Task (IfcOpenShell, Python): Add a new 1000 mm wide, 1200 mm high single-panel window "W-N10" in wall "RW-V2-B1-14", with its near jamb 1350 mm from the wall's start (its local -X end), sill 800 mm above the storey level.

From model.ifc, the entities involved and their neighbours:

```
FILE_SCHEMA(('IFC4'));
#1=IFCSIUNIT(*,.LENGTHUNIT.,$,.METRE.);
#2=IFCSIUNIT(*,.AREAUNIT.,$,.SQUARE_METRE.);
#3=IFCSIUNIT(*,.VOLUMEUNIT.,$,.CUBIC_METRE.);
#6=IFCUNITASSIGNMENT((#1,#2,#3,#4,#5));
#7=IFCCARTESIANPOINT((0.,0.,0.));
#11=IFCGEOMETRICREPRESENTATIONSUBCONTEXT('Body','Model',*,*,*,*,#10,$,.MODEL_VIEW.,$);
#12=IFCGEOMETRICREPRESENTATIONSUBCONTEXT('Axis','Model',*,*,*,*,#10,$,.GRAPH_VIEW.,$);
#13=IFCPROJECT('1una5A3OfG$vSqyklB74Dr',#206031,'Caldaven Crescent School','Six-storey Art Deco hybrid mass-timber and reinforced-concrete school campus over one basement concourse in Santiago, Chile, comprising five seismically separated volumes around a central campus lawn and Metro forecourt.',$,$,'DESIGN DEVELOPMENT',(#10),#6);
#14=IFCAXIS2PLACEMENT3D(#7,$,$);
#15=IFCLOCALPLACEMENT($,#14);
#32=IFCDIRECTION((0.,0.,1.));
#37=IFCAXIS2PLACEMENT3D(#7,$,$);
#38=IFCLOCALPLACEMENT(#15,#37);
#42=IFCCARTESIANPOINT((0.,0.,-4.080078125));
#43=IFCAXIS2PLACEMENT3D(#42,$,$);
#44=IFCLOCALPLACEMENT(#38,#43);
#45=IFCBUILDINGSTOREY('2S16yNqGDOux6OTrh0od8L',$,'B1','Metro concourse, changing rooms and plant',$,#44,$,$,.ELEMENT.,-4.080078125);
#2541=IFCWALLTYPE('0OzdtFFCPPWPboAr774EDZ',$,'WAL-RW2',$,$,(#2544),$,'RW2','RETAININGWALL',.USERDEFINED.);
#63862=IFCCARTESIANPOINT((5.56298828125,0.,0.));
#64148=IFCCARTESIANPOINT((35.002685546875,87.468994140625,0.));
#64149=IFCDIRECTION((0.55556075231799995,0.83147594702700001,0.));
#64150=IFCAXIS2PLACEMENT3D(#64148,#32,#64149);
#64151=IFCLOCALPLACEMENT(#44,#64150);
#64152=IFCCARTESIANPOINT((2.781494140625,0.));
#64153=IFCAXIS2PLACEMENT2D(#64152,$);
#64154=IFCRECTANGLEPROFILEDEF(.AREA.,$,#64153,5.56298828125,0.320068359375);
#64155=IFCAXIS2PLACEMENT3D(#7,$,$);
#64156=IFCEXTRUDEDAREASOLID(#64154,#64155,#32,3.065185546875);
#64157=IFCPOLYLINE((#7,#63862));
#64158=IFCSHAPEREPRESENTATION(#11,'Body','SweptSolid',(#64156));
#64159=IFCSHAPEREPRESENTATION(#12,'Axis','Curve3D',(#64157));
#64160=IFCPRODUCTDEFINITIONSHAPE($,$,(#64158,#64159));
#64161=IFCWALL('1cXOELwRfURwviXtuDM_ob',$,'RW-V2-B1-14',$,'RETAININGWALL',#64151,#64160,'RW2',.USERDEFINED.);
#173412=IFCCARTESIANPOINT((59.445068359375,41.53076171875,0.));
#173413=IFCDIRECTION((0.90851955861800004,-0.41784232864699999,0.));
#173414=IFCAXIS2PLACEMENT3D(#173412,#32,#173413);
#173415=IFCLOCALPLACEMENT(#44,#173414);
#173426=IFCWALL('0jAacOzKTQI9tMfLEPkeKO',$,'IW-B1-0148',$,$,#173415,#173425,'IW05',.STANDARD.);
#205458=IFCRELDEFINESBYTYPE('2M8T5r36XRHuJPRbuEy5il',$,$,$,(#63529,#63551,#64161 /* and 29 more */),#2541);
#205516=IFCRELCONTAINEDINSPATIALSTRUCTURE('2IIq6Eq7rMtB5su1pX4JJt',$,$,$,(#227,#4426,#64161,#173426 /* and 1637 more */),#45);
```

```python
import numpy as np
import ifcopenshell
import ifcopenshell.api.feature
import ifcopenshell.api.geometry
import ifcopenshell.api.root
import ifcopenshell.api.spatial
import ifcopenshell.geom
import ifcopenshell.util.element
import ifcopenshell.util.placement
import ifcopenshell.util.representation
import ifcopenshell.util.shape
import ifcopenshell.util.unit

model = ifcopenshell.open("model.ifc")
unit_scale = ifcopenshell.util.unit.calculate_unit_scale(model)
settings = ifcopenshell.geom.settings()


def volume(element):
    """Net volume in cubic metres, openings subtracted."""
    shape = ifcopenshell.geom.create_shape(settings, element)
    return ifcopenshell.util.shape.get_volume(shape.geometry)


wall = model.by_guid("1cXOELwRfURwviXtuDM_ob")
storey = ifcopenshell.util.element.get_container(wall, ifc_class="IfcBuildingStorey")
context = ifcopenshell.util.representation.get_context(model, "Model", "Body", "MODEL_VIEW")
before = volume(wall)

width, height, from_end, sill = 1, 1.2, 1.35, 0.8  # metres

# The wall runs along its own X axis, and the end named is its -X end.
wall_shape = ifcopenshell.geom.create_shape(settings, wall)
x, y, z = ifcopenshell.util.shape.get_vertices(wall_shape.geometry).T
start = x.min() + from_end
face, thickness = float(y.min()), float(y.max() - y.min())
wall_matrix = ifcopenshell.util.placement.get_local_placement(wall.ObjectPlacement)
level = ifcopenshell.util.placement.get_local_placement(storey.ObjectPlacement)[2, 3]


def in_wall(x, y):
    """Placement at x, y metres in the wall's axes, at sill height."""
    matrix = wall_matrix.copy()
    matrix[:, 3] = wall_matrix @ np.array([x / unit_scale, y / unit_scale, 0.0, 1.0])
    matrix[2, 3] = level + sill / unit_scale
    return matrix


# Opening: a box that overshoots both wall faces by 50 mm.
opening = ifcopenshell.api.root.create_entity(model, ifc_class="IfcOpeningElement", predefined_type="OPENING")
box = ifcopenshell.api.geometry.add_wall_representation(
    model, context=context, length=width, height=height, thickness=thickness + 0.1
)
ifcopenshell.api.geometry.assign_representation(model, product=opening, representation=box)
ifcopenshell.api.geometry.edit_object_placement(model, product=opening, matrix=in_wall(start, face - 0.05), is_si=False)
ifcopenshell.api.feature.add_feature(model, feature=opening, element=wall)

window = ifcopenshell.api.root.create_entity(model, ifc_class="IfcWindow", name="W-N10", predefined_type="WINDOW")
window.OverallWidth, window.OverallHeight = width / unit_scale, height / unit_scale
window.PartitioningType = "SINGLE_PANEL"
body = ifcopenshell.api.geometry.add_window_representation(
    model,
    context=context,
    overall_width=window.OverallWidth,
    overall_height=window.OverallHeight,
    partition_type="SINGLE_PANEL",
)
ifcopenshell.api.geometry.assign_representation(model, product=window, representation=body)
ifcopenshell.api.spatial.assign_container(model, products=[window], relating_structure=storey)
ifcopenshell.api.feature.add_filling(model, opening=opening, element=window)

# Centre the window in the wall's thickness.
ifcopenshell.api.geometry.edit_object_placement(model, product=window, matrix=in_wall(start, face), is_si=False)
window_shape = ifcopenshell.geom.create_shape(settings, window)
depth = ifcopenshell.util.shape.get_vertices(window_shape.geometry)[:, 1]
offset = face + thickness / 2 - (depth.min() + depth.max()) / 2
ifcopenshell.api.geometry.edit_object_placement(model, product=window, matrix=in_wall(start, offset), is_si=False)

after = volume(wall)

print(f"wall volume {before:.3f} -> {after:.3f} m3")

model.write("model_v2.ifc")
```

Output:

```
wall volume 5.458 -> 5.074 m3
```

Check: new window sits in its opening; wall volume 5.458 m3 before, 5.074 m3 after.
